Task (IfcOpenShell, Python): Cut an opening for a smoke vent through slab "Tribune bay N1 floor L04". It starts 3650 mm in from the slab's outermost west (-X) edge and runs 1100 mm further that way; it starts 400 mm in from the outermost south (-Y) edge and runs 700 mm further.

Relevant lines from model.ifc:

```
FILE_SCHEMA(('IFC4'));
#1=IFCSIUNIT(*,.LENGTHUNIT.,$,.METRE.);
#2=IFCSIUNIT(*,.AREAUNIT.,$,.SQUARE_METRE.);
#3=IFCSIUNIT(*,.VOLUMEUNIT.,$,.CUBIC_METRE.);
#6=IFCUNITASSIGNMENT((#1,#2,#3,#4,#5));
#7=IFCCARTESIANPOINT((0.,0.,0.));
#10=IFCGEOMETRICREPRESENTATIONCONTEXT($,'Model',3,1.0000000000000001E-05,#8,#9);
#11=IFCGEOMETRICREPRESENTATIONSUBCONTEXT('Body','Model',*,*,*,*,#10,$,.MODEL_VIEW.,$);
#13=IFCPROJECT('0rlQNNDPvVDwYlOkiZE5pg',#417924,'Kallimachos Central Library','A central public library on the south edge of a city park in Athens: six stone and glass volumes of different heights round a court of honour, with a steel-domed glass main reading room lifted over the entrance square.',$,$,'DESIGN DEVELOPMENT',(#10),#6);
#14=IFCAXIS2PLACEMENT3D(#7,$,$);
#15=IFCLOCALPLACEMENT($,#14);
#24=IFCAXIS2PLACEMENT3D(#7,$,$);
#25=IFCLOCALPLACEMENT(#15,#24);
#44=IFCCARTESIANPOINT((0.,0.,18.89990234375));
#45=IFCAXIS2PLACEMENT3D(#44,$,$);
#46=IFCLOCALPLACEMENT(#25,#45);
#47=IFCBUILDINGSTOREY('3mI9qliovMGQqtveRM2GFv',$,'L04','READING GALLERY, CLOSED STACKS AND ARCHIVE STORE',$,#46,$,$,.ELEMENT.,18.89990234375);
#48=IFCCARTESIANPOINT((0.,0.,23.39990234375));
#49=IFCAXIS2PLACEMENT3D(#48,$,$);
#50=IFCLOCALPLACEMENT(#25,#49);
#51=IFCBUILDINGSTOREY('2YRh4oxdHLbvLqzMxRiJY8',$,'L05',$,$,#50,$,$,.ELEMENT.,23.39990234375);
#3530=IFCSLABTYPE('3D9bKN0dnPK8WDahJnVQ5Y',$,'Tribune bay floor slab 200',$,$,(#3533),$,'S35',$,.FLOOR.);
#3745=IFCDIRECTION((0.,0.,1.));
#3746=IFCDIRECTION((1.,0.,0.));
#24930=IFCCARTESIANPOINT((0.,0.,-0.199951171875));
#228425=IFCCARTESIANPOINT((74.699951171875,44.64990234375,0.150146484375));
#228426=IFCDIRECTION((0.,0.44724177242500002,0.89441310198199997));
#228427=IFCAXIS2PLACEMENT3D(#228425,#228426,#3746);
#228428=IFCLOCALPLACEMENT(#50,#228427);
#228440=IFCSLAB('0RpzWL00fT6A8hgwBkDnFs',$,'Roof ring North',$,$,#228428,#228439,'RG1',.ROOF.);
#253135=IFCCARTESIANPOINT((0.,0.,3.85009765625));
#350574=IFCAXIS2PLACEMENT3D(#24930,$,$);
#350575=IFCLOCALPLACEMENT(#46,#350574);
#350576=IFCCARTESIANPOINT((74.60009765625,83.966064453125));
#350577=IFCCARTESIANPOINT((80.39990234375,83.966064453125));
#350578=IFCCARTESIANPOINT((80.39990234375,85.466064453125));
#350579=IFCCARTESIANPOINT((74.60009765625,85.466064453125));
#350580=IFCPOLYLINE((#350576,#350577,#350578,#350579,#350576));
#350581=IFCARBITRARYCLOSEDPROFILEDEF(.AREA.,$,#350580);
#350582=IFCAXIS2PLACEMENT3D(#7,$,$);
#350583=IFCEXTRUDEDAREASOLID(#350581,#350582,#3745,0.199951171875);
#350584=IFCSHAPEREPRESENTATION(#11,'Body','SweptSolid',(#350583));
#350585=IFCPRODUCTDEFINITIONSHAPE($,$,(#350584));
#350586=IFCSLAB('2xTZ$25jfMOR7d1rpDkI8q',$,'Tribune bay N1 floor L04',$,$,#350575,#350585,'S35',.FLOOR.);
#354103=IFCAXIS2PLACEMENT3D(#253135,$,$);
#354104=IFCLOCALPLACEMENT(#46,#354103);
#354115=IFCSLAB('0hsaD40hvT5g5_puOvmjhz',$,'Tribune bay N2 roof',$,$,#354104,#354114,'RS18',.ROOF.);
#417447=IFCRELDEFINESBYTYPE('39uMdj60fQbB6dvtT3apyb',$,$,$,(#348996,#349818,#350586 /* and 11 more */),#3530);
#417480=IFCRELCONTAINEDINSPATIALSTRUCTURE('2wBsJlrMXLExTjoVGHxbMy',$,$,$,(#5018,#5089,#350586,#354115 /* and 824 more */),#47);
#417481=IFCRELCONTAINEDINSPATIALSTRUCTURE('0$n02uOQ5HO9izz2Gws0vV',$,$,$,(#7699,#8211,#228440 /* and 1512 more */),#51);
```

```python
import numpy as np
import ifcopenshell
import ifcopenshell.api.feature
import ifcopenshell.api.geometry
import ifcopenshell.api.root
import ifcopenshell.geom
import ifcopenshell.util.placement
import ifcopenshell.util.representation
import ifcopenshell.util.shape
import ifcopenshell.util.unit

model = ifcopenshell.open("model.ifc")
unit_scale = ifcopenshell.util.unit.calculate_unit_scale(model)
settings = ifcopenshell.geom.settings()


def volume(element):
    """Net volume in cubic metres, openings subtracted."""
    shape = ifcopenshell.geom.create_shape(settings, element)
    return ifcopenshell.util.shape.get_volume(shape.geometry)


slab = model.by_id(350586)
before = volume(slab)

# Extent in the slab's own axes, in metres. The edges named are its -X and -Y sides.
slab_shape = ifcopenshell.geom.create_shape(settings, slab)
vertices = ifcopenshell.util.shape.get_vertices(slab_shape.geometry)
x_min, y_min, bottom = vertices.min(axis=0)
top = vertices[:, 2].max()

opening = ifcopenshell.api.root.create_entity(model, ifc_class="IfcOpeningElement", name="Smoke vent opening", predefined_type="OPENING")
context = ifcopenshell.util.representation.get_context(model, "Model", "Body", "MODEL_VIEW")
width, depth = 1.1, 0.7
outline = [(0.0, 0.0), (width, 0.0), (width, depth), (0.0, depth), (0.0, 0.0)]
# Overshoot both faces by 50 mm so the cut is clean.
shape = ifcopenshell.api.geometry.add_slab_representation(
    model, context=context, depth=top - bottom + 0.1, polyline=outline
)
ifcopenshell.api.geometry.assign_representation(model, product=opening, representation=shape)

matrix = ifcopenshell.util.placement.get_local_placement(slab.ObjectPlacement)
matrix[:, 3] = matrix @ np.append(np.array([x_min + 3.65, y_min + 0.4, bottom - 0.05]) / unit_scale, 1.0)
ifcopenshell.api.geometry.edit_object_placement(model, product=opening, matrix=matrix, is_si=False)
ifcopenshell.api.feature.add_feature(model, feature=opening, element=slab)

after = volume(slab)

print(f"slab volume {before:.3f} -> {after:.3f} m3")

model.write("model_rev.ifc")
```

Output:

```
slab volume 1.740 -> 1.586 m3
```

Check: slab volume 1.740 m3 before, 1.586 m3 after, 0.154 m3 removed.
